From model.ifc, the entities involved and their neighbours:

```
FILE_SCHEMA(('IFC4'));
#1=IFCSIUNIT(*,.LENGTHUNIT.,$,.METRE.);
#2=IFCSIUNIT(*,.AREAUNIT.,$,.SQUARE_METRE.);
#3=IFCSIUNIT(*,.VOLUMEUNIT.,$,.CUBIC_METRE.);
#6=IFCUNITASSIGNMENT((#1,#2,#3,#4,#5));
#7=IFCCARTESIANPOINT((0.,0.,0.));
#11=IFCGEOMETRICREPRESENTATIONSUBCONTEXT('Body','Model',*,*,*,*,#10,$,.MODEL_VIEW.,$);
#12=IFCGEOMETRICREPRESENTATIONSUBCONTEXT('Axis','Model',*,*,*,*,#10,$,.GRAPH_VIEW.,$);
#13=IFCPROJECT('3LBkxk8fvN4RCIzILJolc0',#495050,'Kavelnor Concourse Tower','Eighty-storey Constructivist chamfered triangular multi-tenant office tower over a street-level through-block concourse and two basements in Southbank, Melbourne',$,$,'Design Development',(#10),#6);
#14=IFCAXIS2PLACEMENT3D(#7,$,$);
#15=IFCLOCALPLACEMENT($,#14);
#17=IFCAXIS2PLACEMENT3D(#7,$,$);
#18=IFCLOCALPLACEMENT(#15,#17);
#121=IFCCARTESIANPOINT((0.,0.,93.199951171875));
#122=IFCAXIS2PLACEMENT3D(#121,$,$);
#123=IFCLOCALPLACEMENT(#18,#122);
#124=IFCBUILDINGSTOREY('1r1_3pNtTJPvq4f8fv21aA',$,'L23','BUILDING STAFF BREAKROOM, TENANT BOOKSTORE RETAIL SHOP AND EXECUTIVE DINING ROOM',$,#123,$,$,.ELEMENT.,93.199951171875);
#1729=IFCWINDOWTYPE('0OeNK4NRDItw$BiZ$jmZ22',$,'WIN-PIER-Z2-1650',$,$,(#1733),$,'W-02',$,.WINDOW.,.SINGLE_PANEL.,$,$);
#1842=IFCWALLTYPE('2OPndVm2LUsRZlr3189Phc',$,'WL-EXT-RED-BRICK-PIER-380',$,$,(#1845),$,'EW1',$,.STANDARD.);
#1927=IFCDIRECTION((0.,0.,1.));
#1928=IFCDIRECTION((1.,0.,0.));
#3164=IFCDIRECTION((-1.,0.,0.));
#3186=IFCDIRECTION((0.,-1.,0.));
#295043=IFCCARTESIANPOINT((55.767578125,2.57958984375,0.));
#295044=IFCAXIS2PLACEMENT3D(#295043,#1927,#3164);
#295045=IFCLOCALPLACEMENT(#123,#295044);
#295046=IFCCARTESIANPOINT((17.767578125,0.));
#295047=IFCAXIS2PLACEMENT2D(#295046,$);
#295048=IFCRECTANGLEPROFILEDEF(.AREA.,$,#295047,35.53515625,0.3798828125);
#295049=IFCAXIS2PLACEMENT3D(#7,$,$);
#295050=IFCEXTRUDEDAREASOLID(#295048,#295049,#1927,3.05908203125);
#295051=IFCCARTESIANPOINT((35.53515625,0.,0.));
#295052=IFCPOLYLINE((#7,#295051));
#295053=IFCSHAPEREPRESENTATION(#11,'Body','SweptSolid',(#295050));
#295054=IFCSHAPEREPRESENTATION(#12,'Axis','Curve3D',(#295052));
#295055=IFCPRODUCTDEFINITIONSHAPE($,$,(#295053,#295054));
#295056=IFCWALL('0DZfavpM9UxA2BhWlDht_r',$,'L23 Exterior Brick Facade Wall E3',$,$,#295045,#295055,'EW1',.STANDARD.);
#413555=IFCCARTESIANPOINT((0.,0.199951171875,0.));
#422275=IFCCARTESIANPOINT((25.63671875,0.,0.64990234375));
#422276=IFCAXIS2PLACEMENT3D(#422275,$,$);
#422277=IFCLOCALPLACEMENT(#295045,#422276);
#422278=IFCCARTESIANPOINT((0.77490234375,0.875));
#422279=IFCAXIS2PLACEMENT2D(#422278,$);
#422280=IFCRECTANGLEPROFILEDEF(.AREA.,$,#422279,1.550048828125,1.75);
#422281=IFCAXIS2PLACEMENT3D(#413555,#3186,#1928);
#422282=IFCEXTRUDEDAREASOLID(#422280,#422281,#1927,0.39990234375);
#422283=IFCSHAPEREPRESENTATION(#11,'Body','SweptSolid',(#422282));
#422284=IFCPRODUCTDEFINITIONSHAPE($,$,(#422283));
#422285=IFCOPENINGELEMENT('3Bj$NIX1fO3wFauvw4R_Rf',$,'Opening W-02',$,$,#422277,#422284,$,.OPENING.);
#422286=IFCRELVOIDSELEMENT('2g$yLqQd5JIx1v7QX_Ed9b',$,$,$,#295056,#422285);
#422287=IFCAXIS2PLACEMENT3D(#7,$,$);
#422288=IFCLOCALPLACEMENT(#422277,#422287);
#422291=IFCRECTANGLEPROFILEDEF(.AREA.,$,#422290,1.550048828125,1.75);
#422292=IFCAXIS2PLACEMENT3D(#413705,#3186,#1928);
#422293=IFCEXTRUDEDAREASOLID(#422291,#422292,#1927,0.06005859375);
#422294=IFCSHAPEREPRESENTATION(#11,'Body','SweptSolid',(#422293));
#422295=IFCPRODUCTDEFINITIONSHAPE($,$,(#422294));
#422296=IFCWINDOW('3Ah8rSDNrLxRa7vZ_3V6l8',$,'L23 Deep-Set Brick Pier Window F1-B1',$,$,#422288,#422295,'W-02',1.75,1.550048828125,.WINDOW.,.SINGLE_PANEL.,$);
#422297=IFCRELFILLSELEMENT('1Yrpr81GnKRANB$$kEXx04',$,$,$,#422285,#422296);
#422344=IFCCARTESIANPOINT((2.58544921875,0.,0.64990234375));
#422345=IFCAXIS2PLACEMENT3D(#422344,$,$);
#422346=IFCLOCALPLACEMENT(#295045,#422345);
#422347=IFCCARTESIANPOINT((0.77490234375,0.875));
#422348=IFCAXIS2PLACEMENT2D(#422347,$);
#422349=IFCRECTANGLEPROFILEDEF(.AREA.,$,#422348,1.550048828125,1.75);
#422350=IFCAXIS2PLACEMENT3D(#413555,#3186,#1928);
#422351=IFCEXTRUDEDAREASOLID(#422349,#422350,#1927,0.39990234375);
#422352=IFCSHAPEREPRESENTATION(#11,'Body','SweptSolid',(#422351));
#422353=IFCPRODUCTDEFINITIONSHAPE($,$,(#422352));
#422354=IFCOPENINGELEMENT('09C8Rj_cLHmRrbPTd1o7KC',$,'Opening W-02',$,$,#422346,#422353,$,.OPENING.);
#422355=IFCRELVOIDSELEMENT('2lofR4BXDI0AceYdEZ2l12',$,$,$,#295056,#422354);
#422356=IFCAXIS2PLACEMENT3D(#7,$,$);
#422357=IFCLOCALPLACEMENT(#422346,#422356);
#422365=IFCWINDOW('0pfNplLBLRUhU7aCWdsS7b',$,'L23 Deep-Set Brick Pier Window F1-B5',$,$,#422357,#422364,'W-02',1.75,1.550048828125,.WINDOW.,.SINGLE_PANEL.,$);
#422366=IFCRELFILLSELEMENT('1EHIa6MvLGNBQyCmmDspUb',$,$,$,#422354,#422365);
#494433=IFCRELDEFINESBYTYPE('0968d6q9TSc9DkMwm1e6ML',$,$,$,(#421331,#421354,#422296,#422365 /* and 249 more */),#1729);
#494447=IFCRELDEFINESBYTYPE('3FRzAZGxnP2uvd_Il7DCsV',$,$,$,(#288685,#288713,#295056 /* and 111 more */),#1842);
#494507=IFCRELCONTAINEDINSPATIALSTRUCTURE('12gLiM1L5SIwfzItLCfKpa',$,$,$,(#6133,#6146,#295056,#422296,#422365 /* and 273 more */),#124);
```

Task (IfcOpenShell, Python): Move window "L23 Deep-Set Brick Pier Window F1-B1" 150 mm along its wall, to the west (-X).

```python
import ifcopenshell
import ifcopenshell.api.geometry
import ifcopenshell.util.placement
import ifcopenshell.util.unit

model = ifcopenshell.open("model.ifc")
unit_scale = ifcopenshell.util.unit.calculate_unit_scale(model)

window = model.by_id(422296)
opening = window.FillsVoids[0].RelatingOpeningElement
wall = opening.VoidsElements[0].RelatingBuildingElement

wall_matrix = ifcopenshell.util.placement.get_local_placement(wall.ObjectPlacement)
shift = wall_matrix[:3, 0] * 0.15 / unit_scale
before = ifcopenshell.util.placement.get_local_placement(window.ObjectPlacement)[:3, 3].copy()

# The window is placed relative to its opening, so it follows when the opening moves.
matrix = ifcopenshell.util.placement.get_local_placement(opening.ObjectPlacement)
matrix[:3, 3] += shift
ifcopenshell.api.geometry.edit_object_placement(
    model, product=opening, matrix=matrix, is_si=False, should_transform_children=True
)

after = ifcopenshell.util.placement.get_local_placement(window.ObjectPlacement)[:3, 3]
print("window moved by", (after - before).round(3) + 0.0)

model.write("model_v2.ifc")
```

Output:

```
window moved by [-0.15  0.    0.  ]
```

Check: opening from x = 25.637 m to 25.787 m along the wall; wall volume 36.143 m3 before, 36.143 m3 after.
